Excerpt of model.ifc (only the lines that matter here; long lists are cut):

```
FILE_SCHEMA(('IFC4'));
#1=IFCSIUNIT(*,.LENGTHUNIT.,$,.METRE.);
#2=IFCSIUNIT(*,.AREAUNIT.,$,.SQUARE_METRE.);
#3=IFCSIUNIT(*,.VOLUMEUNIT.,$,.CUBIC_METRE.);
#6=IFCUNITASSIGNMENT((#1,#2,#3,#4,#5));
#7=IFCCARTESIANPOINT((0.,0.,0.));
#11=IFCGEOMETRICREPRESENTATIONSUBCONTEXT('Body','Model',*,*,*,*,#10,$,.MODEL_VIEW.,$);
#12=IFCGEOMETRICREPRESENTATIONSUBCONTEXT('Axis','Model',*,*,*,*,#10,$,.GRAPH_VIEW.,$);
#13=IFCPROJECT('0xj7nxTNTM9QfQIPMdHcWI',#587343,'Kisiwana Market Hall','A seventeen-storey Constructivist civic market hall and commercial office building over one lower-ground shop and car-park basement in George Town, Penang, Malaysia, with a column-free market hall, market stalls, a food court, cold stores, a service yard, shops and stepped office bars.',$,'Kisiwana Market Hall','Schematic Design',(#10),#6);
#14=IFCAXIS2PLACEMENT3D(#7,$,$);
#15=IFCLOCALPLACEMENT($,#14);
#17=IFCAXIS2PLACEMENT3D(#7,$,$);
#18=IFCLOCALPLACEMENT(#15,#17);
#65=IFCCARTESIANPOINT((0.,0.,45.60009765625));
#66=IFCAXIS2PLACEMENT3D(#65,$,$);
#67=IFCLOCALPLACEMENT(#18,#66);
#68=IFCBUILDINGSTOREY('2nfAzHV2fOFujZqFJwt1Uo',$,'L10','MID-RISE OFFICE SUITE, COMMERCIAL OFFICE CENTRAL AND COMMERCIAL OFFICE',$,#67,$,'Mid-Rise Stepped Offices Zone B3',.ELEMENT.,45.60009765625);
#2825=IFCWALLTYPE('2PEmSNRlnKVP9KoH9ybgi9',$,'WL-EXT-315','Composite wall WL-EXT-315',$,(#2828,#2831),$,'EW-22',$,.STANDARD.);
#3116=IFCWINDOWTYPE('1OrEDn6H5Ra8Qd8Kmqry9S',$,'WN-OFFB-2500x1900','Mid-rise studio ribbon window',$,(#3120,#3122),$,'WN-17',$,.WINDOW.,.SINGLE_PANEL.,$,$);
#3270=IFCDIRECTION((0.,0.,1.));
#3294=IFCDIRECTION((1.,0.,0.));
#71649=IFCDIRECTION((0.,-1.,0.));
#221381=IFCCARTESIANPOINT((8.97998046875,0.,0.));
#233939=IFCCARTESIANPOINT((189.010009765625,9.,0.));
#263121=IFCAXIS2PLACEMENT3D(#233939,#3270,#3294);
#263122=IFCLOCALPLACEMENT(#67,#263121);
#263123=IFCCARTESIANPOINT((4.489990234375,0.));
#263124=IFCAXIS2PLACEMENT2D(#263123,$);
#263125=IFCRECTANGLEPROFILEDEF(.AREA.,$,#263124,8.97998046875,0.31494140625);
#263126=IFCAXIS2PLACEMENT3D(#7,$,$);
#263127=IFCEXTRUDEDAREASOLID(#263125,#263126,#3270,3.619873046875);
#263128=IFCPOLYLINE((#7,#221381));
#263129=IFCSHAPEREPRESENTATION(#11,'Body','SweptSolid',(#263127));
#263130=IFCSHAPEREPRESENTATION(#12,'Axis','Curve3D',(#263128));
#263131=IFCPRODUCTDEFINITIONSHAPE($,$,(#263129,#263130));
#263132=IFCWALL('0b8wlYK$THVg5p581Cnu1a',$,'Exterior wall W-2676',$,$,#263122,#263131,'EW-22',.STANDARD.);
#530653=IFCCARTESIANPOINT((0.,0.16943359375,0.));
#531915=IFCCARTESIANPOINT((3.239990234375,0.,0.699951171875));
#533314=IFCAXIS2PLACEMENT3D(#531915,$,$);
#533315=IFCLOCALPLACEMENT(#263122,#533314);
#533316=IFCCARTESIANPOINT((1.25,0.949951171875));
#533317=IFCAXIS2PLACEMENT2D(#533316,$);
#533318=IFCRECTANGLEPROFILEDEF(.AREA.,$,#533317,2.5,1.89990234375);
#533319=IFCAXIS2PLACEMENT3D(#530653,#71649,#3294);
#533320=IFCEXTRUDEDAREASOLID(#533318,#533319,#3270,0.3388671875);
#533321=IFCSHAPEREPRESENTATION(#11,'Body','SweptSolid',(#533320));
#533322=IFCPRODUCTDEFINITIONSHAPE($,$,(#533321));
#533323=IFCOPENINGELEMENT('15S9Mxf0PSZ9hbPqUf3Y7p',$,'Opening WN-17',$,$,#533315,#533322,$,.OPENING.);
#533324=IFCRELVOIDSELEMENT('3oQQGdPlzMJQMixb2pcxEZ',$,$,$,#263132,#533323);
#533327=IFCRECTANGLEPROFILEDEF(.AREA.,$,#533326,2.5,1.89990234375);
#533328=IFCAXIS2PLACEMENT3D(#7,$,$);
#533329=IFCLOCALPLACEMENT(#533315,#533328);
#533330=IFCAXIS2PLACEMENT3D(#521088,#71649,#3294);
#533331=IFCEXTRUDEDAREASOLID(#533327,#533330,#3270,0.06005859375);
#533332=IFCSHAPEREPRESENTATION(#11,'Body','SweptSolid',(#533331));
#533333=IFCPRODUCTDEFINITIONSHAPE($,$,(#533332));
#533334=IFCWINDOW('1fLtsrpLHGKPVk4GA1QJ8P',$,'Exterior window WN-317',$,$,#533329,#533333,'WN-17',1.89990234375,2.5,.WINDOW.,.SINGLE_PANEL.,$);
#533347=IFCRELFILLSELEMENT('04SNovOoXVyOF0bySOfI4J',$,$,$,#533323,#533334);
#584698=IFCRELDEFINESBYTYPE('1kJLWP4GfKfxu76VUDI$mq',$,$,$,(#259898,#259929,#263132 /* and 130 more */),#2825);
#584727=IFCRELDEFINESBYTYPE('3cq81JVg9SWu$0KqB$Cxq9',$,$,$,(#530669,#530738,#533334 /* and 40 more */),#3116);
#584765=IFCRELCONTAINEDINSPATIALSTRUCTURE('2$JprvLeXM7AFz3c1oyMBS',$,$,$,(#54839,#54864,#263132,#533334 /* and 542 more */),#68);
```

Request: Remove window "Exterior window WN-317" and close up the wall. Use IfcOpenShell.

```python
import ifcopenshell
import ifcopenshell.api.feature
import ifcopenshell.api.root
import ifcopenshell.geom
import ifcopenshell.util.shape

model = ifcopenshell.open("model.ifc")
settings = ifcopenshell.geom.settings()


def volume(element):
    """Net volume in cubic metres, openings subtracted."""
    shape = ifcopenshell.geom.create_shape(settings, element)
    return ifcopenshell.util.shape.get_volume(shape.geometry)


window = model.by_guid("1fLtsrpLHGKPVk4GA1QJ8P")
opening = window.FillsVoids[0].RelatingOpeningElement
wall = opening.VoidsElements[0].RelatingBuildingElement
before = volume(wall)

ifcopenshell.api.root.remove_product(model, product=window)
ifcopenshell.api.feature.remove_feature(model, feature=opening)

after = volume(wall)

print(f"wall volume {before:.3f} -> {after:.3f} m3")

model.write("model-out.ifc")
```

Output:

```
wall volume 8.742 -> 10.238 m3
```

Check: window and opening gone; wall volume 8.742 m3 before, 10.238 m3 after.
